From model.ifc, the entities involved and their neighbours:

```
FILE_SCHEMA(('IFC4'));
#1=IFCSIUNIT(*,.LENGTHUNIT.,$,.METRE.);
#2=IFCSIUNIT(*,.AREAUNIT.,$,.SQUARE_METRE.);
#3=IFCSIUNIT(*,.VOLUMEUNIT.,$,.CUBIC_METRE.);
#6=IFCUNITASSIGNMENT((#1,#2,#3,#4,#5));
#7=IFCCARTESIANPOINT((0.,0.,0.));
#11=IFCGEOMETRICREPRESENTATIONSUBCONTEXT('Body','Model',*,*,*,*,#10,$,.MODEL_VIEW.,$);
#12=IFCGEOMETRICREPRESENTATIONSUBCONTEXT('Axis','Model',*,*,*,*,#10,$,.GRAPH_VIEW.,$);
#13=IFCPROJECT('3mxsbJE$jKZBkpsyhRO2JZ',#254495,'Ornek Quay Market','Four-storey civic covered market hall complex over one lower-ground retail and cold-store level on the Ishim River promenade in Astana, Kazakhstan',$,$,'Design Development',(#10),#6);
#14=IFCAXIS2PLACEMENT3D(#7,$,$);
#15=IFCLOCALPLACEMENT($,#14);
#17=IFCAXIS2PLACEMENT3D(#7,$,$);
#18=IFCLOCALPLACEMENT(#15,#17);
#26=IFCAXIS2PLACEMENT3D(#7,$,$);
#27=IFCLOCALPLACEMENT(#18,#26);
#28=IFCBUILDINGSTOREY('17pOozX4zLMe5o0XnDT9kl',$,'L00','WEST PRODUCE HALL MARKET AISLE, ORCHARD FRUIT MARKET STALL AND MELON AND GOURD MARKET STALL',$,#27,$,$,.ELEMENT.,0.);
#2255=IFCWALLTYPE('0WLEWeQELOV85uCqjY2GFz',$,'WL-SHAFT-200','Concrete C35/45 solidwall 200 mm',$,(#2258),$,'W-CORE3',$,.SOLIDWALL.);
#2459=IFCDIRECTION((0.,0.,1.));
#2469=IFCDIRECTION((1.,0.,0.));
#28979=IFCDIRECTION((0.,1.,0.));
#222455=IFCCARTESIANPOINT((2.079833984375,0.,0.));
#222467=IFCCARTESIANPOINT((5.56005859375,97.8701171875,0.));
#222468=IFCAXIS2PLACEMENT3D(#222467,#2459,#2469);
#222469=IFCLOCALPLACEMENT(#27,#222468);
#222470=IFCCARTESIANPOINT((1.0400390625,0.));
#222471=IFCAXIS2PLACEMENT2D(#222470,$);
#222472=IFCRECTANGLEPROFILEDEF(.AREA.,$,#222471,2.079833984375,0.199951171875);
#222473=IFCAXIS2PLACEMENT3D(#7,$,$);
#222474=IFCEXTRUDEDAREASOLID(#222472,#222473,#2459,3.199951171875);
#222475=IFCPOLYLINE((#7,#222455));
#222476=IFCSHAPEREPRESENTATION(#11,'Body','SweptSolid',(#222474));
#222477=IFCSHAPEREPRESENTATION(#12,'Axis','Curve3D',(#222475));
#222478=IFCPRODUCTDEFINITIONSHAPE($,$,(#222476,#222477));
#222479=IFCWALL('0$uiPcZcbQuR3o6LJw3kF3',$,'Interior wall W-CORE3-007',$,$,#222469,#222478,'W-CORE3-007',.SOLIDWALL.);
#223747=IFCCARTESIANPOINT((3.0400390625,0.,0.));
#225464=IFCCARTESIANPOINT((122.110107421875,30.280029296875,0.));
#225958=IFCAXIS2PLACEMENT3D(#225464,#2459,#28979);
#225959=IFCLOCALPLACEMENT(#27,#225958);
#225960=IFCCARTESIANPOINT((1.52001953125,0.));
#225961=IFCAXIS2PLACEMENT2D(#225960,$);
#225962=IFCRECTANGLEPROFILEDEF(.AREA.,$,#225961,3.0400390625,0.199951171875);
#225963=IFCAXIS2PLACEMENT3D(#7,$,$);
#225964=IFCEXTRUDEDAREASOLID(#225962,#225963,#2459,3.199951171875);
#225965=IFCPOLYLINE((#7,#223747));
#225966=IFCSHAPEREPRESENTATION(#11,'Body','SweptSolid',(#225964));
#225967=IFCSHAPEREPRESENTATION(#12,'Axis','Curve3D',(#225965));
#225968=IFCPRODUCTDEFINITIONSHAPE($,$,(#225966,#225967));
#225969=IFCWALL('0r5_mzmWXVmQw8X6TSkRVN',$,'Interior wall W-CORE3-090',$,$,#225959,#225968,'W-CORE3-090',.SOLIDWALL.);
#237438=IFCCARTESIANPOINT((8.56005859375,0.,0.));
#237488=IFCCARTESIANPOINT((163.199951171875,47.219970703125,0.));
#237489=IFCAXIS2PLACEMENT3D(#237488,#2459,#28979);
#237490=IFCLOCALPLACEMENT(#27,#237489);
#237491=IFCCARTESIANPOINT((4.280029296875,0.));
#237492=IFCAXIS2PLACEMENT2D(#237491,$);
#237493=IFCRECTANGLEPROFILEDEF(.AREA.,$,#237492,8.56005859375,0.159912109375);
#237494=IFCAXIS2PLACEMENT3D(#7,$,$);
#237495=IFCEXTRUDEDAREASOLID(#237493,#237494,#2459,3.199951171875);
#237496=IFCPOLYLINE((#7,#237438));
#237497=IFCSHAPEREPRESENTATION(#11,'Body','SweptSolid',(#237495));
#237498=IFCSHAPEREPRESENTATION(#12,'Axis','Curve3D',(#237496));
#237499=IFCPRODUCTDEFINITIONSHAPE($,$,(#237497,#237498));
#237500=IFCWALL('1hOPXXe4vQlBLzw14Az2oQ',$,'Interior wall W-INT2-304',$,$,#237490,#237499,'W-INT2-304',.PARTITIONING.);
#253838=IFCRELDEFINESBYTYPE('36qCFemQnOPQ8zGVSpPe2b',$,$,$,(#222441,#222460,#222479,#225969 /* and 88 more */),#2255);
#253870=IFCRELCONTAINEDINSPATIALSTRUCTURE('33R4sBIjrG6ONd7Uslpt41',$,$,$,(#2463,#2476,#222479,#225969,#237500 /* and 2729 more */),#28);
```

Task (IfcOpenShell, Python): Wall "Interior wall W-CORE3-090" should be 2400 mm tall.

```python
import ifcopenshell
import ifcopenshell.geom
import ifcopenshell.util.representation
import ifcopenshell.util.shape

model = ifcopenshell.open("model.ifc")
settings = ifcopenshell.geom.settings()


def volume(element):
    """Net volume in cubic metres, openings subtracted."""
    shape = ifcopenshell.geom.create_shape(settings, element)
    return ifcopenshell.util.shape.get_volume(shape.geometry)


wall = model.by_guid("0r5_mzmWXVmQw8X6TSkRVN")
before = volume(wall)

body = ifcopenshell.util.representation.get_representation(wall, "Model", "Body")
solid = body.Items[0]
old_height = solid.Depth
solid.Depth = 2.4
after = volume(wall)

print(f"height {old_height:g} -> {solid.Depth:g}, volume {before:.3f} -> {after:.3f} m3")

model.write("model_edited.ifc")
```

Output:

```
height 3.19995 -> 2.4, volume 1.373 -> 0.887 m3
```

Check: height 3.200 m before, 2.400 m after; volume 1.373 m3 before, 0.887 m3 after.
